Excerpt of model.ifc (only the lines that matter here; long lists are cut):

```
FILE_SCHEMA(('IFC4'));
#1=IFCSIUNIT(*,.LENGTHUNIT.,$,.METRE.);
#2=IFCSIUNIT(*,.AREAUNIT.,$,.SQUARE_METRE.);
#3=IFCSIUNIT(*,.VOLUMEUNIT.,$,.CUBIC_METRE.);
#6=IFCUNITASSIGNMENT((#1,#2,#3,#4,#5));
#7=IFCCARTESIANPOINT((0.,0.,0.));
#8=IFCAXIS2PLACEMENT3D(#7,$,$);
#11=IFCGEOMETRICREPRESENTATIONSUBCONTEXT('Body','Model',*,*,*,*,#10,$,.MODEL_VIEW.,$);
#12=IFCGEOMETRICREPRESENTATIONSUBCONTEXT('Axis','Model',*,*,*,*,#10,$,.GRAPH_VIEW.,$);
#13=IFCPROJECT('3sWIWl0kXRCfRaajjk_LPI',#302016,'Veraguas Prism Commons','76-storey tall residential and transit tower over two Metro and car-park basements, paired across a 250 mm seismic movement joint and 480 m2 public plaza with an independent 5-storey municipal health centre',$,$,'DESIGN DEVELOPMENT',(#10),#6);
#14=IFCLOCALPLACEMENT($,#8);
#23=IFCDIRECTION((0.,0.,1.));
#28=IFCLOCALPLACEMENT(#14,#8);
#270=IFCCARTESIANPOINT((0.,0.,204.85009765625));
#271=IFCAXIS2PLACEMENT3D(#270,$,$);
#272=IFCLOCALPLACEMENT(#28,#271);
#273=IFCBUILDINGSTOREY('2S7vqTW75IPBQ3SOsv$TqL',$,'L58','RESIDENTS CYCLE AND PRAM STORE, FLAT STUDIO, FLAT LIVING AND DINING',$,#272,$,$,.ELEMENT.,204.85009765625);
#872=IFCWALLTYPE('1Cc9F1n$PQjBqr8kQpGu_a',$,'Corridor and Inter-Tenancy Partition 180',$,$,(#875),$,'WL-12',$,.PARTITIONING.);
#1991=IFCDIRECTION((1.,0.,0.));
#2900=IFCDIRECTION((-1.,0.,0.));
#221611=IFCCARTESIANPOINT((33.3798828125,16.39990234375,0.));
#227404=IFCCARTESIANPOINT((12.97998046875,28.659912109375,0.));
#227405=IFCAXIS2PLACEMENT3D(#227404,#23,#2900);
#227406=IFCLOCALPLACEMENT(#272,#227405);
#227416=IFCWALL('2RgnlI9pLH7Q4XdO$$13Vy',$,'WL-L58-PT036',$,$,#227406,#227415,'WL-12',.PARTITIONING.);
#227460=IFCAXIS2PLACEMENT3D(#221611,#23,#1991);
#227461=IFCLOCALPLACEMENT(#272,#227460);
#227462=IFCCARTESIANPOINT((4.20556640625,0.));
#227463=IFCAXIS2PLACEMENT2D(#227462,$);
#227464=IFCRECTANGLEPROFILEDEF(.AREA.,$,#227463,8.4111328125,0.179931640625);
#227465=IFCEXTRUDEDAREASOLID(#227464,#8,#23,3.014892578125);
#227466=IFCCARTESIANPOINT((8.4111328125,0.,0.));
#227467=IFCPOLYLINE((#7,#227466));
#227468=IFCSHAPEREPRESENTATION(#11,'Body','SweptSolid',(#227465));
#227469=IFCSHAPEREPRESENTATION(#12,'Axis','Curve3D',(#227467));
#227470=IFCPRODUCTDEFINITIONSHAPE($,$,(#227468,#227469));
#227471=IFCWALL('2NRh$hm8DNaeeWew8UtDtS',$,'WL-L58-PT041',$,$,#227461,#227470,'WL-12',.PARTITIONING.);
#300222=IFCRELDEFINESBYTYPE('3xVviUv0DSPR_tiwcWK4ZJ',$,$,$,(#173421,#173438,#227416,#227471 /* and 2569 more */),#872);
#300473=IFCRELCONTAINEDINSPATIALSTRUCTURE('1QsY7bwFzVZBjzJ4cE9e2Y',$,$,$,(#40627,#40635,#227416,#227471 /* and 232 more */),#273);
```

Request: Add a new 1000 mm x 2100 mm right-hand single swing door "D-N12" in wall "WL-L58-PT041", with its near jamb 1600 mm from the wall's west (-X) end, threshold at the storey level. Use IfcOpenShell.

```python
import numpy as np
import ifcopenshell
import ifcopenshell.api.feature
import ifcopenshell.api.geometry
import ifcopenshell.api.root
import ifcopenshell.api.spatial
import ifcopenshell.geom
import ifcopenshell.util.element
import ifcopenshell.util.placement
import ifcopenshell.util.representation
import ifcopenshell.util.shape
import ifcopenshell.util.unit

model = ifcopenshell.open("model.ifc")
unit_scale = ifcopenshell.util.unit.calculate_unit_scale(model)
settings = ifcopenshell.geom.settings()


def volume(element):
    """Net volume in cubic metres, openings subtracted."""
    shape = ifcopenshell.geom.create_shape(settings, element)
    return ifcopenshell.util.shape.get_volume(shape.geometry)


wall = model.by_guid("2NRh$hm8DNaeeWew8UtDtS")
storey = ifcopenshell.util.element.get_container(wall, ifc_class="IfcBuildingStorey")
context = ifcopenshell.util.representation.get_context(model, "Model", "Body", "MODEL_VIEW")
before = volume(wall)

width, height, from_end, sill = 1, 2.1, 1.6, 0.0  # metres

# The wall runs along its own X axis, and the end named is its -X end.
wall_shape = ifcopenshell.geom.create_shape(settings, wall)
x, y, z = ifcopenshell.util.shape.get_vertices(wall_shape.geometry).T
start = x.min() + from_end
face, thickness = float(y.min()), float(y.max() - y.min())
wall_matrix = ifcopenshell.util.placement.get_local_placement(wall.ObjectPlacement)
level = ifcopenshell.util.placement.get_local_placement(storey.ObjectPlacement)[2, 3]


def in_wall(x, y):
    """Placement at x, y metres in the wall's axes, at sill height."""
    matrix = wall_matrix.copy()
    matrix[:, 3] = wall_matrix @ np.array([x / unit_scale, y / unit_scale, 0.0, 1.0])
    matrix[2, 3] = level + sill / unit_scale
    return matrix


# Opening: a box that overshoots both wall faces by 50 mm.
opening = ifcopenshell.api.root.create_entity(model, ifc_class="IfcOpeningElement", predefined_type="OPENING")
box = ifcopenshell.api.geometry.add_wall_representation(
    model, context=context, length=width, height=height, thickness=thickness + 0.1
)
ifcopenshell.api.geometry.assign_representation(model, product=opening, representation=box)
ifcopenshell.api.geometry.edit_object_placement(model, product=opening, matrix=in_wall(start, face - 0.05), is_si=False)
ifcopenshell.api.feature.add_feature(model, feature=opening, element=wall)

door = ifcopenshell.api.root.create_entity(model, ifc_class="IfcDoor", name="D-N12", predefined_type="DOOR")
door.OverallWidth, door.OverallHeight = width / unit_scale, height / unit_scale
door.OperationType = "SINGLE_SWING_RIGHT"
body = ifcopenshell.api.geometry.add_door_representation(
    model,
    context=context,
    overall_width=door.OverallWidth,
    overall_height=door.OverallHeight,
    operation_type="SINGLE_SWING_RIGHT",
    lining_properties={"LiningDepth": thickness / unit_scale, "ThresholdDepth": thickness / unit_scale},
)
ifcopenshell.api.geometry.assign_representation(model, product=door, representation=body)
ifcopenshell.api.spatial.assign_container(model, products=[door], relating_structure=storey)
ifcopenshell.api.feature.add_filling(model, opening=opening, element=door)

# The lining spans the wall, so the door starts at the wall face.
ifcopenshell.api.geometry.edit_object_placement(model, product=door, matrix=in_wall(start, face), is_si=False)

after = volume(wall)

print(f"wall volume {before:.3f} -> {after:.3f} m3")

model.write("model-out.ifc")
```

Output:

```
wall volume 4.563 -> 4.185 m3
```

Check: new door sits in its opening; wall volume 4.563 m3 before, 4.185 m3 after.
